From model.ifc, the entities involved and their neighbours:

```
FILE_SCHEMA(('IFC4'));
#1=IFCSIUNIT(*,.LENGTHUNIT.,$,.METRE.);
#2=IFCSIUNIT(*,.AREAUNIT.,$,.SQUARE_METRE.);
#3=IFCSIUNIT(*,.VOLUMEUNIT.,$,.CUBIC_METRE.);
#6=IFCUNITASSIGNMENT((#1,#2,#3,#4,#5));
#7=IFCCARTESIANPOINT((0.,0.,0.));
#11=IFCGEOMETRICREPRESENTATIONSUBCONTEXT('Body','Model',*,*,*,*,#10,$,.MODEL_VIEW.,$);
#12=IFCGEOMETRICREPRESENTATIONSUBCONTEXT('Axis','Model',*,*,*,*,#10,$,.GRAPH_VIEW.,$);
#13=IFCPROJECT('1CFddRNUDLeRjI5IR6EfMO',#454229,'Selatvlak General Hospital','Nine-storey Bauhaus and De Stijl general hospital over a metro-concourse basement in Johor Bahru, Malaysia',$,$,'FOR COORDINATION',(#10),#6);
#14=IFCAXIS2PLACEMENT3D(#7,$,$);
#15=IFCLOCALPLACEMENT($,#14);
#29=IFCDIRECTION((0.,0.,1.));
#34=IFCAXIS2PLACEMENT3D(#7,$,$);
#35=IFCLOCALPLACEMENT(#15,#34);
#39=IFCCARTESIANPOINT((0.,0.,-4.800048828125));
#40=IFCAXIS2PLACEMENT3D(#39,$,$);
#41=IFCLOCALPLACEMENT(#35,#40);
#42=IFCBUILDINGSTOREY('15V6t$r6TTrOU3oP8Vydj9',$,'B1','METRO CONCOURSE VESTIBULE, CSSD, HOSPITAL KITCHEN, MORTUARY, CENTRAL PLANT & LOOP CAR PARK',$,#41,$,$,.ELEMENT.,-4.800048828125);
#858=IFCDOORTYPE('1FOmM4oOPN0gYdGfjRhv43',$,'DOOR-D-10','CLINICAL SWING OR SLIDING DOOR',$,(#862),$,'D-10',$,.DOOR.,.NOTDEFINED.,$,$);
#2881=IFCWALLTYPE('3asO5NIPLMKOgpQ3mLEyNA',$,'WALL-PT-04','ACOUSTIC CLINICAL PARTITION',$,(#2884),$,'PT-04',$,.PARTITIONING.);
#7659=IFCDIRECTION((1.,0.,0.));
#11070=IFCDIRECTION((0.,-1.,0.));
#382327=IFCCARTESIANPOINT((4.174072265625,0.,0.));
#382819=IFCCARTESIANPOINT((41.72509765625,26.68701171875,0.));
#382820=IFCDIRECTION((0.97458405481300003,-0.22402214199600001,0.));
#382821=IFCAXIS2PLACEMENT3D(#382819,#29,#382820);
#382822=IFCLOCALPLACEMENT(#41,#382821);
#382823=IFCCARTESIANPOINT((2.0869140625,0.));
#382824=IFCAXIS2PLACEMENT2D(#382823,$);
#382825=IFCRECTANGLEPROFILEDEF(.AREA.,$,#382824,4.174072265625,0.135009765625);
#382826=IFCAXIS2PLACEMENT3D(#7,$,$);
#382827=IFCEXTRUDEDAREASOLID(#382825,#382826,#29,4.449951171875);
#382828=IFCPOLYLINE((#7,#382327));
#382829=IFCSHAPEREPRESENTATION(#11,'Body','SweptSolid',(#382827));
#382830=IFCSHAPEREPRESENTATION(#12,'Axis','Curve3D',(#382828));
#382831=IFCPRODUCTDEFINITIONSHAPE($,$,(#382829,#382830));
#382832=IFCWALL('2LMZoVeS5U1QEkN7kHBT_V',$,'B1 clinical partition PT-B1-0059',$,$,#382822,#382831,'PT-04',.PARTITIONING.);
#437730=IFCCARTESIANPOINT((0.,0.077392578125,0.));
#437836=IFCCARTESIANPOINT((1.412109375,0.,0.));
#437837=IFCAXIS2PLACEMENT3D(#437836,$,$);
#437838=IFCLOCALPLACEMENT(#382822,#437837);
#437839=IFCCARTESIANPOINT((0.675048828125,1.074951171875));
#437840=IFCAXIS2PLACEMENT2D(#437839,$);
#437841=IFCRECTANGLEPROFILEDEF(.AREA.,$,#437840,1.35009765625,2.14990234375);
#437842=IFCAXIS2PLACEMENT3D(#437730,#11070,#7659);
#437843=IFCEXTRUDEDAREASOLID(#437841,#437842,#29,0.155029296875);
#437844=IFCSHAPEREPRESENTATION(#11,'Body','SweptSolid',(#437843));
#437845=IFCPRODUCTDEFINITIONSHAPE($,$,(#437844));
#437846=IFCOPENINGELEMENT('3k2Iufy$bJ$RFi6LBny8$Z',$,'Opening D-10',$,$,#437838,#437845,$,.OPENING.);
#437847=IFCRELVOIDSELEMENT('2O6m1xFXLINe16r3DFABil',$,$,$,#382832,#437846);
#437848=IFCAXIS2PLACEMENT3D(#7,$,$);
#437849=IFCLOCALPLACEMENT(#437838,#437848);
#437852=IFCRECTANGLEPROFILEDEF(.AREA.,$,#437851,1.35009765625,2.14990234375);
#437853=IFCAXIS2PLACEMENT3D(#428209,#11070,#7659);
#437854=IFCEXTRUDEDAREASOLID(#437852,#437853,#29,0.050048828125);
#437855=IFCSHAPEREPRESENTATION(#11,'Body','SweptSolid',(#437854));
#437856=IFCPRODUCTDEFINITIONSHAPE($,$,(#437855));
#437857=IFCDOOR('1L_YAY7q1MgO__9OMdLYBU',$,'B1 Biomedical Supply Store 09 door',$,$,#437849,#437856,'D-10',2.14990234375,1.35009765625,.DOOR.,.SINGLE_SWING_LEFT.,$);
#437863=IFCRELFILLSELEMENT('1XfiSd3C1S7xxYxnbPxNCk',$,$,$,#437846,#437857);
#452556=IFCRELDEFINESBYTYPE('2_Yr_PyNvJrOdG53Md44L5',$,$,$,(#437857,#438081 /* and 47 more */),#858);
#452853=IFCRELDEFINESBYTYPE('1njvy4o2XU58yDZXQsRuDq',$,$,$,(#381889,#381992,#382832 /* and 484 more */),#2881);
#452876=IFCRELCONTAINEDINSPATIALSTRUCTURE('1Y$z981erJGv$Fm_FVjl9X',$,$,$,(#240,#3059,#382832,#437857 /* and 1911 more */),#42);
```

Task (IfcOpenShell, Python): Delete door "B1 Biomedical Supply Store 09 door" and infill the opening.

```python
import ifcopenshell
import ifcopenshell.api.feature
import ifcopenshell.api.root
import ifcopenshell.geom
import ifcopenshell.util.shape

model = ifcopenshell.open("model.ifc")
settings = ifcopenshell.geom.settings()


def volume(element):
    """Net volume in cubic metres, openings subtracted."""
    shape = ifcopenshell.geom.create_shape(settings, element)
    return ifcopenshell.util.shape.get_volume(shape.geometry)


door = model.by_id(437857)
opening = door.FillsVoids[0].RelatingOpeningElement
wall = opening.VoidsElements[0].RelatingBuildingElement
before = volume(wall)

ifcopenshell.api.root.remove_product(model, product=door)
ifcopenshell.api.feature.remove_feature(model, feature=opening)

after = volume(wall)

print(f"wall volume {before:.3f} -> {after:.3f} m3")

model.write("model_edited.ifc")
```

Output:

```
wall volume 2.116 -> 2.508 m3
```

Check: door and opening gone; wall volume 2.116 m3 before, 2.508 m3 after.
